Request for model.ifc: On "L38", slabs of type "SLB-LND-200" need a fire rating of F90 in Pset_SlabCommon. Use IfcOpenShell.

First a look at what the model holds.

```python
import ifcopenshell
import ifcopenshell.util.element

model = ifcopenshell.open("model.ifc")
print(model.schema)
storey = next(s for s in model.by_type("IfcBuildingStorey") if s.Name == "L38")
slabs = [e for e in ifcopenshell.util.element.get_decomposition(storey) if e.is_a("IfcSlab")]
seen = {}
for e in slabs:
    element_type = ifcopenshell.util.element.get_type(e)
    key = (element_type.Name if element_type != e and element_type else None, ifcopenshell.util.element.get_pset(e, "Pset_SlabCommon", "FireRating"))
    seen[key] = seen.get(key, 0) + 1
for (name, value), count in sorted(seen.items(), key=str):
    print(count, "x", name, "|", value)
```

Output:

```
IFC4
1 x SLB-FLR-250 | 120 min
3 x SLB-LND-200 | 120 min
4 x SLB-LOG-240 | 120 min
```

```python
import ifcopenshell
import ifcopenshell.api.pset
import ifcopenshell.util.element

model = ifcopenshell.open("model.ifc")

storey = next(s for s in model.by_type("IfcBuildingStorey") if s.Name == "L38")
slabs = [e for e in ifcopenshell.util.element.get_decomposition(storey) if e.is_a("IfcSlab")]

count = 0
for e in slabs:
    element_type = ifcopenshell.util.element.get_type(e)
    if element_type in (None, e) or element_type.Name != "SLB-LND-200":
        continue
    # add_pset returns the element's existing set when there is one.
    pset = ifcopenshell.api.pset.add_pset(model, product=e, name="Pset_SlabCommon")
    ifcopenshell.api.pset.edit_pset(model, pset=pset, properties={"FireRating": "F90"})
    count += 1

print(count, "slabs updated")

model.write("model_updated.ifc")
```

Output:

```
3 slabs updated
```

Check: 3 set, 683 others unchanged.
